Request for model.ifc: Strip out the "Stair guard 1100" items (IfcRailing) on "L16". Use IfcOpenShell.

First a look at what the model holds.

```python
import ifcopenshell
import ifcopenshell.util.element

model = ifcopenshell.open("model.ifc")
print(model.schema)
storey = next(s for s in model.by_type("IfcBuildingStorey") if s.Name == "L16")
railings = [e for e in ifcopenshell.util.element.get_decomposition(storey) if e.is_a("IfcRailing")]
seen = {}
for e in railings:
    element_type = ifcopenshell.util.element.get_type(e)
    name = element_type.Name if element_type not in (None, e) else None
    seen[name] = seen.get(name, 0) + 1
for name, count in sorted(seen.items(), key=str):
    print(count, "x", name)
```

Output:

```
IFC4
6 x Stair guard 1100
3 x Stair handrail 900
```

```python
import ifcopenshell
import ifcopenshell.api.root
import ifcopenshell.util.element

model = ifcopenshell.open("model.ifc")

storey = next(s for s in model.by_type("IfcBuildingStorey") if s.Name == "L16")
railings = [e for e in ifcopenshell.util.element.get_decomposition(storey) if e.is_a("IfcRailing")]
targets = [e for e in railings if (t := ifcopenshell.util.element.get_type(e)) not in (None, e) and t.Name == "Stair guard 1100"]

for e in targets:
    ifcopenshell.api.root.remove_product(model, product=e)
print(len(targets), "removed")

model.write("model_edited.ifc")
```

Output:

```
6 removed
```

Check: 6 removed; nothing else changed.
